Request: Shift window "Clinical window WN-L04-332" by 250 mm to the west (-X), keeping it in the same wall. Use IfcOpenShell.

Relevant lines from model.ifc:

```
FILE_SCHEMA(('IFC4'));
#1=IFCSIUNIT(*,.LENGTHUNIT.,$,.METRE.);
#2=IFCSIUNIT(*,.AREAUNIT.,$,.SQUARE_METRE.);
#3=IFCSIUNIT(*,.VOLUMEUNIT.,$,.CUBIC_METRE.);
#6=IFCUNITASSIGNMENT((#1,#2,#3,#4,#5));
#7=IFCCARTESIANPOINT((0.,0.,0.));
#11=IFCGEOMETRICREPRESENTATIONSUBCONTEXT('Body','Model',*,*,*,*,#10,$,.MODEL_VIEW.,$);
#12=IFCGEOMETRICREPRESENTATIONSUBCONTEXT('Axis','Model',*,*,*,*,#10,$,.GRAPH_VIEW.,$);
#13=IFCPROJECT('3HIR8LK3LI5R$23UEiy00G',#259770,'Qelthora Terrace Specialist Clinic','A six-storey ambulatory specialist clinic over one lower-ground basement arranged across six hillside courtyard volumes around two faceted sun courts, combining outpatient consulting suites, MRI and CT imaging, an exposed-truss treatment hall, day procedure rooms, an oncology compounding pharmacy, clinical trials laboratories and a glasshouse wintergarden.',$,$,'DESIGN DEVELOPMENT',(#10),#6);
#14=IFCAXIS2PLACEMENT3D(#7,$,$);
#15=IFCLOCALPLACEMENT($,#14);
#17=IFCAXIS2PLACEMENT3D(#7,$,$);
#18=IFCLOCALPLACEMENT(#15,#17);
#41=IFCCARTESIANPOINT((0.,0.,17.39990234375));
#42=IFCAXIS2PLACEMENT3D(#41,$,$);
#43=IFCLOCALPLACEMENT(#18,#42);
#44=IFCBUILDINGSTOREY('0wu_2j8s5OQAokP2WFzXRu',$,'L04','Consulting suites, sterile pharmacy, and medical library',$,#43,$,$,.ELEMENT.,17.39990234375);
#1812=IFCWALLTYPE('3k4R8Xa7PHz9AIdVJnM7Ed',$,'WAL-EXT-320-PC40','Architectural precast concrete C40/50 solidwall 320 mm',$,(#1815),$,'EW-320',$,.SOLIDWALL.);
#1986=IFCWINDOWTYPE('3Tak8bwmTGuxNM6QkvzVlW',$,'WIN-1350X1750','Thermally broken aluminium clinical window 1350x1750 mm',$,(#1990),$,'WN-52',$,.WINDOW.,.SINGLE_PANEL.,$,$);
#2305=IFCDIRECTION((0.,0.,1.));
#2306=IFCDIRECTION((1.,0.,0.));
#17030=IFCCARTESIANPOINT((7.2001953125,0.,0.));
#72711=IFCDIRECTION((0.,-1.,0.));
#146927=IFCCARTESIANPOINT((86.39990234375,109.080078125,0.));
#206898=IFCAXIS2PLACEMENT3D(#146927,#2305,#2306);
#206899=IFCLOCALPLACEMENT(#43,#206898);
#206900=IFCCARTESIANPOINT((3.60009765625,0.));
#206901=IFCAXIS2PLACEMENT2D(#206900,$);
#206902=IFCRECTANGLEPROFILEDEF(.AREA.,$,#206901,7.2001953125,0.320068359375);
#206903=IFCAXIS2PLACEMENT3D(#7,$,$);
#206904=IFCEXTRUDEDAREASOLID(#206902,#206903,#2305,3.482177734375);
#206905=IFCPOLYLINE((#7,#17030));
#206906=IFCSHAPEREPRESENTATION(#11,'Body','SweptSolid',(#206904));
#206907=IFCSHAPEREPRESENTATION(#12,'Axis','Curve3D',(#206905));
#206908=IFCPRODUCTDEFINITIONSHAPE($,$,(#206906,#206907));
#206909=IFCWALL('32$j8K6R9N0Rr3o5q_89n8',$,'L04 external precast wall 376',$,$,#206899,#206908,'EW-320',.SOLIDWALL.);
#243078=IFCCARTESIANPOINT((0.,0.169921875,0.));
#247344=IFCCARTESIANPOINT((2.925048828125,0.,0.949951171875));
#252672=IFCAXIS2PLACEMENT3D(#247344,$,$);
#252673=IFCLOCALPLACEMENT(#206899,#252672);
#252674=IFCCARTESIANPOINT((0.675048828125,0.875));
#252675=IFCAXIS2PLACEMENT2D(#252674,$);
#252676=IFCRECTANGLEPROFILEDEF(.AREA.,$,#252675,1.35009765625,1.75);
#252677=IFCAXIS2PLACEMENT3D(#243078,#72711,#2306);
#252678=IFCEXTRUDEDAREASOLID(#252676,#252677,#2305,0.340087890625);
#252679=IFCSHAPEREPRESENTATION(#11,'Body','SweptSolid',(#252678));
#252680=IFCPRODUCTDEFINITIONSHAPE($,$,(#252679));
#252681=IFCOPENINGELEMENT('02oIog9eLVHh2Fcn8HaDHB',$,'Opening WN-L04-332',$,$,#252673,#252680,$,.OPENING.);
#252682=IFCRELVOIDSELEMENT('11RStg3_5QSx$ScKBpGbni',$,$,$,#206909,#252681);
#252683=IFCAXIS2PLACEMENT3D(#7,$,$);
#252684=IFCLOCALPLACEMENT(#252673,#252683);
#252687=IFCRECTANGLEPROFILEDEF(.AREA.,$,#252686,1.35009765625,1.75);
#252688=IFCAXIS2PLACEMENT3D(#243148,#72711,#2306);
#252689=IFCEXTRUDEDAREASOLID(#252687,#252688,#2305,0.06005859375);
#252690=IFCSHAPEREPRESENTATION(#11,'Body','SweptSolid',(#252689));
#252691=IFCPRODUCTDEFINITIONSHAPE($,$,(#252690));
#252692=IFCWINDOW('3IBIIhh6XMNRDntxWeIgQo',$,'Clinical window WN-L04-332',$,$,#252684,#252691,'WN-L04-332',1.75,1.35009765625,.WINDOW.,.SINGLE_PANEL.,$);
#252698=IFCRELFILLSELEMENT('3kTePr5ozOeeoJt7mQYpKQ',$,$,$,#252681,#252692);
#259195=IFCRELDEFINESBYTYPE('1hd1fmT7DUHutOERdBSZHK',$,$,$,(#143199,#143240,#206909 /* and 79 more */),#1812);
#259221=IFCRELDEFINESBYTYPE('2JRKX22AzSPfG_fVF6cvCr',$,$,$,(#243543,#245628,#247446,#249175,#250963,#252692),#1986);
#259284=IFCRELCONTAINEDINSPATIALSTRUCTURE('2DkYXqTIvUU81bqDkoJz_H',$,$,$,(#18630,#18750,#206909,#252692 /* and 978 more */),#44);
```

```python
import ifcopenshell
import ifcopenshell.api.geometry
import ifcopenshell.util.placement

model = ifcopenshell.open("model.ifc")

window = model.by_guid("3IBIIhh6XMNRDntxWeIgQo")
opening = window.FillsVoids[0].RelatingOpeningElement
wall = opening.VoidsElements[0].RelatingBuildingElement

wall_matrix = ifcopenshell.util.placement.get_local_placement(wall.ObjectPlacement)
shift = wall_matrix[:3, 0] * -0.25
before = ifcopenshell.util.placement.get_local_placement(window.ObjectPlacement)[:3, 3].copy()

# The window is placed relative to its opening, so it follows when the opening moves.
matrix = ifcopenshell.util.placement.get_local_placement(opening.ObjectPlacement)
matrix[:3, 3] += shift
ifcopenshell.api.geometry.edit_object_placement(
    model, product=opening, matrix=matrix, is_si=False, should_transform_children=True
)

after = ifcopenshell.util.placement.get_local_placement(window.ObjectPlacement)[:3, 3]
print("window moved by", (after - before).round(3) + 0.0)

model.write("model-out.ifc")
```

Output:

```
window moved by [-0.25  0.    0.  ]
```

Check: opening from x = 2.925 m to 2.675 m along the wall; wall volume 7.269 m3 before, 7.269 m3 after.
